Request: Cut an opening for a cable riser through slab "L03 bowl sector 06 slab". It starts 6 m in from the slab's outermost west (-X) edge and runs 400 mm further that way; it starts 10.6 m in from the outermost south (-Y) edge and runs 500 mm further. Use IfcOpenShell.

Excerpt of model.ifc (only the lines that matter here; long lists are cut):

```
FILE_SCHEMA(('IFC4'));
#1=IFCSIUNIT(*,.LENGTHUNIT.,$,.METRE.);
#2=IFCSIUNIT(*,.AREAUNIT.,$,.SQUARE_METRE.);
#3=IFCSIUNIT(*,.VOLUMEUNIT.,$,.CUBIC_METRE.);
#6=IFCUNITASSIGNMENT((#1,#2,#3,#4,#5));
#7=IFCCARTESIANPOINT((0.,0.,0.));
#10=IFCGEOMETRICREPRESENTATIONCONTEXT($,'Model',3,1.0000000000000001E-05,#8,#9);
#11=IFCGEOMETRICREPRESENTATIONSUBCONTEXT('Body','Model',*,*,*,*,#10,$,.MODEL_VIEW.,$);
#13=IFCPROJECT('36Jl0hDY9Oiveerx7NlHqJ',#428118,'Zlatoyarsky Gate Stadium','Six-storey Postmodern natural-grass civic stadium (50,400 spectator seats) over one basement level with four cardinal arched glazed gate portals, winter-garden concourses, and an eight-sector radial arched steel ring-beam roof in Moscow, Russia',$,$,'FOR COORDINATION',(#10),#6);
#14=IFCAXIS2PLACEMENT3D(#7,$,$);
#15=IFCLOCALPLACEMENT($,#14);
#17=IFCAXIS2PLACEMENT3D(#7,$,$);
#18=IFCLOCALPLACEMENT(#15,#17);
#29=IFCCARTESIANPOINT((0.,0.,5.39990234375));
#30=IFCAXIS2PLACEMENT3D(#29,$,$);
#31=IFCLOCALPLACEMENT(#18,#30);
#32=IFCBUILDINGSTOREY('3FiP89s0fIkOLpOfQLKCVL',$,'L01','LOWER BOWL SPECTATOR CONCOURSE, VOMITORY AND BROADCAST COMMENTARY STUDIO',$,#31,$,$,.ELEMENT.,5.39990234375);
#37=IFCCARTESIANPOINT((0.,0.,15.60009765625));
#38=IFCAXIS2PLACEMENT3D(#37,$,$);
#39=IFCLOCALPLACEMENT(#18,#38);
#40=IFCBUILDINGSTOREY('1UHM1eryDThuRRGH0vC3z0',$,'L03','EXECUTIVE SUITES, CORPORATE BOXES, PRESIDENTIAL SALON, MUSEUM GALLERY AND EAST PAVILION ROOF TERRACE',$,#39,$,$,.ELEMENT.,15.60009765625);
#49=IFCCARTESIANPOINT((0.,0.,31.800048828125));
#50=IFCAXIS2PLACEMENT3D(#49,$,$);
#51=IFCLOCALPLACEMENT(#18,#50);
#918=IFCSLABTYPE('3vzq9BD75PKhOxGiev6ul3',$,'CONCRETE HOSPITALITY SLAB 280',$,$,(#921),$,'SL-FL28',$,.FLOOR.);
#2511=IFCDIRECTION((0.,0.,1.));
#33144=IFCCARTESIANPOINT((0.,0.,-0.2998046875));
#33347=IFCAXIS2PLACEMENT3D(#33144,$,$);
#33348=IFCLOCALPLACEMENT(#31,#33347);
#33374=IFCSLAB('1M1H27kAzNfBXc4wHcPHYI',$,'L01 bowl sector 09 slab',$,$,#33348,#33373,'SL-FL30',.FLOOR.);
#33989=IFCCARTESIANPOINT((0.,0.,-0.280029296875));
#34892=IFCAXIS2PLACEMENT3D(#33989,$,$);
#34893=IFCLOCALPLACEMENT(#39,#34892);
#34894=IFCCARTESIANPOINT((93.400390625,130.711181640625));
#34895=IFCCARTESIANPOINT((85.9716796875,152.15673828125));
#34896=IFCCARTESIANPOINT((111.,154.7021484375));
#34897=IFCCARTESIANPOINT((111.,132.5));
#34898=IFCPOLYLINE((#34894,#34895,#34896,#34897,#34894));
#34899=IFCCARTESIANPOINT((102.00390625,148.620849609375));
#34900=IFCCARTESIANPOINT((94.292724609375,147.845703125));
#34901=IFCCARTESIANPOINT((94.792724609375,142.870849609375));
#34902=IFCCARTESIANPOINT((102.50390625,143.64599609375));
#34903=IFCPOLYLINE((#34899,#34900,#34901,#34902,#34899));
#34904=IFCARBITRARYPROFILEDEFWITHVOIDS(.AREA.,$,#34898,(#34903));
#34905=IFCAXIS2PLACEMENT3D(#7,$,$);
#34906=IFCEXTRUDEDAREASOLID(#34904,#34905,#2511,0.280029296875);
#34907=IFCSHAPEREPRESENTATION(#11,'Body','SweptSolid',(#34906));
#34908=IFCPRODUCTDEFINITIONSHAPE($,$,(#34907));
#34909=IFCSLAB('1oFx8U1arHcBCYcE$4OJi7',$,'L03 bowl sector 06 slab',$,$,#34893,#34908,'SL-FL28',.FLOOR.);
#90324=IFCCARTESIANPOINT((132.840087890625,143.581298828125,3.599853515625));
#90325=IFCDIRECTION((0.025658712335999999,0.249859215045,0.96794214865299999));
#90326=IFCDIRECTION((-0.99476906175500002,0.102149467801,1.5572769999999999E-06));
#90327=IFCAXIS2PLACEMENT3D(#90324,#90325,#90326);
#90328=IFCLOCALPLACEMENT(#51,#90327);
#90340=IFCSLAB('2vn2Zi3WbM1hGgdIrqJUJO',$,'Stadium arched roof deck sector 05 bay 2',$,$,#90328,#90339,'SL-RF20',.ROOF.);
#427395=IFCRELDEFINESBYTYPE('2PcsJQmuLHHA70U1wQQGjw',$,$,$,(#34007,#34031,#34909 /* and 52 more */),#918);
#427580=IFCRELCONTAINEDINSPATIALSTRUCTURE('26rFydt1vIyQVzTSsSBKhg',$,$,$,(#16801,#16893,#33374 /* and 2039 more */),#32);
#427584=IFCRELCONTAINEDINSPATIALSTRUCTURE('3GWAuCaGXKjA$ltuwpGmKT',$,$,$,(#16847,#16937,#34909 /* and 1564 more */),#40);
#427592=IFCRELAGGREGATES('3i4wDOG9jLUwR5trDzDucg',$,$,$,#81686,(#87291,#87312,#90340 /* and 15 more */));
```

```python
import numpy as np
import ifcopenshell
import ifcopenshell.api.feature
import ifcopenshell.api.geometry
import ifcopenshell.api.root
import ifcopenshell.geom
import ifcopenshell.util.placement
import ifcopenshell.util.representation
import ifcopenshell.util.shape
import ifcopenshell.util.unit

model = ifcopenshell.open("model.ifc")
unit_scale = ifcopenshell.util.unit.calculate_unit_scale(model)
settings = ifcopenshell.geom.settings()


def volume(element):
    """Net volume in cubic metres, openings subtracted."""
    shape = ifcopenshell.geom.create_shape(settings, element)
    return ifcopenshell.util.shape.get_volume(shape.geometry)


slab = model.by_guid("1oFx8U1arHcBCYcE$4OJi7")
before = volume(slab)

# Extent in the slab's own axes, in metres. The edges named are its -X and -Y sides.
slab_shape = ifcopenshell.geom.create_shape(settings, slab)
vertices = ifcopenshell.util.shape.get_vertices(slab_shape.geometry)
x_min, y_min, bottom = vertices.min(axis=0)
top = vertices[:, 2].max()

opening = ifcopenshell.api.root.create_entity(model, ifc_class="IfcOpeningElement", name="Cable riser opening", predefined_type="OPENING")
context = ifcopenshell.util.representation.get_context(model, "Model", "Body", "MODEL_VIEW")
width, depth = 0.4, 0.5
outline = [(0.0, 0.0), (width, 0.0), (width, depth), (0.0, depth), (0.0, 0.0)]
# Overshoot both faces by 50 mm so the cut is clean.
shape = ifcopenshell.api.geometry.add_slab_representation(
    model, context=context, depth=top - bottom + 0.1, polyline=outline
)
ifcopenshell.api.geometry.assign_representation(model, product=opening, representation=shape)

matrix = ifcopenshell.util.placement.get_local_placement(slab.ObjectPlacement)
matrix[:, 3] = matrix @ np.append(np.array([x_min + 6, y_min + 10.6, bottom - 0.05]) / unit_scale, 1.0)
ifcopenshell.api.geometry.edit_object_placement(model, product=opening, matrix=matrix, is_si=False)
ifcopenshell.api.feature.add_feature(model, feature=opening, element=slab)

after = volume(slab)

print(f"slab volume {before:.3f} -> {after:.3f} m3")

model.write("model_updated.ifc")
```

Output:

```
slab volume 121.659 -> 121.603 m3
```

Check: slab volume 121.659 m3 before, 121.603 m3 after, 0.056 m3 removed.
